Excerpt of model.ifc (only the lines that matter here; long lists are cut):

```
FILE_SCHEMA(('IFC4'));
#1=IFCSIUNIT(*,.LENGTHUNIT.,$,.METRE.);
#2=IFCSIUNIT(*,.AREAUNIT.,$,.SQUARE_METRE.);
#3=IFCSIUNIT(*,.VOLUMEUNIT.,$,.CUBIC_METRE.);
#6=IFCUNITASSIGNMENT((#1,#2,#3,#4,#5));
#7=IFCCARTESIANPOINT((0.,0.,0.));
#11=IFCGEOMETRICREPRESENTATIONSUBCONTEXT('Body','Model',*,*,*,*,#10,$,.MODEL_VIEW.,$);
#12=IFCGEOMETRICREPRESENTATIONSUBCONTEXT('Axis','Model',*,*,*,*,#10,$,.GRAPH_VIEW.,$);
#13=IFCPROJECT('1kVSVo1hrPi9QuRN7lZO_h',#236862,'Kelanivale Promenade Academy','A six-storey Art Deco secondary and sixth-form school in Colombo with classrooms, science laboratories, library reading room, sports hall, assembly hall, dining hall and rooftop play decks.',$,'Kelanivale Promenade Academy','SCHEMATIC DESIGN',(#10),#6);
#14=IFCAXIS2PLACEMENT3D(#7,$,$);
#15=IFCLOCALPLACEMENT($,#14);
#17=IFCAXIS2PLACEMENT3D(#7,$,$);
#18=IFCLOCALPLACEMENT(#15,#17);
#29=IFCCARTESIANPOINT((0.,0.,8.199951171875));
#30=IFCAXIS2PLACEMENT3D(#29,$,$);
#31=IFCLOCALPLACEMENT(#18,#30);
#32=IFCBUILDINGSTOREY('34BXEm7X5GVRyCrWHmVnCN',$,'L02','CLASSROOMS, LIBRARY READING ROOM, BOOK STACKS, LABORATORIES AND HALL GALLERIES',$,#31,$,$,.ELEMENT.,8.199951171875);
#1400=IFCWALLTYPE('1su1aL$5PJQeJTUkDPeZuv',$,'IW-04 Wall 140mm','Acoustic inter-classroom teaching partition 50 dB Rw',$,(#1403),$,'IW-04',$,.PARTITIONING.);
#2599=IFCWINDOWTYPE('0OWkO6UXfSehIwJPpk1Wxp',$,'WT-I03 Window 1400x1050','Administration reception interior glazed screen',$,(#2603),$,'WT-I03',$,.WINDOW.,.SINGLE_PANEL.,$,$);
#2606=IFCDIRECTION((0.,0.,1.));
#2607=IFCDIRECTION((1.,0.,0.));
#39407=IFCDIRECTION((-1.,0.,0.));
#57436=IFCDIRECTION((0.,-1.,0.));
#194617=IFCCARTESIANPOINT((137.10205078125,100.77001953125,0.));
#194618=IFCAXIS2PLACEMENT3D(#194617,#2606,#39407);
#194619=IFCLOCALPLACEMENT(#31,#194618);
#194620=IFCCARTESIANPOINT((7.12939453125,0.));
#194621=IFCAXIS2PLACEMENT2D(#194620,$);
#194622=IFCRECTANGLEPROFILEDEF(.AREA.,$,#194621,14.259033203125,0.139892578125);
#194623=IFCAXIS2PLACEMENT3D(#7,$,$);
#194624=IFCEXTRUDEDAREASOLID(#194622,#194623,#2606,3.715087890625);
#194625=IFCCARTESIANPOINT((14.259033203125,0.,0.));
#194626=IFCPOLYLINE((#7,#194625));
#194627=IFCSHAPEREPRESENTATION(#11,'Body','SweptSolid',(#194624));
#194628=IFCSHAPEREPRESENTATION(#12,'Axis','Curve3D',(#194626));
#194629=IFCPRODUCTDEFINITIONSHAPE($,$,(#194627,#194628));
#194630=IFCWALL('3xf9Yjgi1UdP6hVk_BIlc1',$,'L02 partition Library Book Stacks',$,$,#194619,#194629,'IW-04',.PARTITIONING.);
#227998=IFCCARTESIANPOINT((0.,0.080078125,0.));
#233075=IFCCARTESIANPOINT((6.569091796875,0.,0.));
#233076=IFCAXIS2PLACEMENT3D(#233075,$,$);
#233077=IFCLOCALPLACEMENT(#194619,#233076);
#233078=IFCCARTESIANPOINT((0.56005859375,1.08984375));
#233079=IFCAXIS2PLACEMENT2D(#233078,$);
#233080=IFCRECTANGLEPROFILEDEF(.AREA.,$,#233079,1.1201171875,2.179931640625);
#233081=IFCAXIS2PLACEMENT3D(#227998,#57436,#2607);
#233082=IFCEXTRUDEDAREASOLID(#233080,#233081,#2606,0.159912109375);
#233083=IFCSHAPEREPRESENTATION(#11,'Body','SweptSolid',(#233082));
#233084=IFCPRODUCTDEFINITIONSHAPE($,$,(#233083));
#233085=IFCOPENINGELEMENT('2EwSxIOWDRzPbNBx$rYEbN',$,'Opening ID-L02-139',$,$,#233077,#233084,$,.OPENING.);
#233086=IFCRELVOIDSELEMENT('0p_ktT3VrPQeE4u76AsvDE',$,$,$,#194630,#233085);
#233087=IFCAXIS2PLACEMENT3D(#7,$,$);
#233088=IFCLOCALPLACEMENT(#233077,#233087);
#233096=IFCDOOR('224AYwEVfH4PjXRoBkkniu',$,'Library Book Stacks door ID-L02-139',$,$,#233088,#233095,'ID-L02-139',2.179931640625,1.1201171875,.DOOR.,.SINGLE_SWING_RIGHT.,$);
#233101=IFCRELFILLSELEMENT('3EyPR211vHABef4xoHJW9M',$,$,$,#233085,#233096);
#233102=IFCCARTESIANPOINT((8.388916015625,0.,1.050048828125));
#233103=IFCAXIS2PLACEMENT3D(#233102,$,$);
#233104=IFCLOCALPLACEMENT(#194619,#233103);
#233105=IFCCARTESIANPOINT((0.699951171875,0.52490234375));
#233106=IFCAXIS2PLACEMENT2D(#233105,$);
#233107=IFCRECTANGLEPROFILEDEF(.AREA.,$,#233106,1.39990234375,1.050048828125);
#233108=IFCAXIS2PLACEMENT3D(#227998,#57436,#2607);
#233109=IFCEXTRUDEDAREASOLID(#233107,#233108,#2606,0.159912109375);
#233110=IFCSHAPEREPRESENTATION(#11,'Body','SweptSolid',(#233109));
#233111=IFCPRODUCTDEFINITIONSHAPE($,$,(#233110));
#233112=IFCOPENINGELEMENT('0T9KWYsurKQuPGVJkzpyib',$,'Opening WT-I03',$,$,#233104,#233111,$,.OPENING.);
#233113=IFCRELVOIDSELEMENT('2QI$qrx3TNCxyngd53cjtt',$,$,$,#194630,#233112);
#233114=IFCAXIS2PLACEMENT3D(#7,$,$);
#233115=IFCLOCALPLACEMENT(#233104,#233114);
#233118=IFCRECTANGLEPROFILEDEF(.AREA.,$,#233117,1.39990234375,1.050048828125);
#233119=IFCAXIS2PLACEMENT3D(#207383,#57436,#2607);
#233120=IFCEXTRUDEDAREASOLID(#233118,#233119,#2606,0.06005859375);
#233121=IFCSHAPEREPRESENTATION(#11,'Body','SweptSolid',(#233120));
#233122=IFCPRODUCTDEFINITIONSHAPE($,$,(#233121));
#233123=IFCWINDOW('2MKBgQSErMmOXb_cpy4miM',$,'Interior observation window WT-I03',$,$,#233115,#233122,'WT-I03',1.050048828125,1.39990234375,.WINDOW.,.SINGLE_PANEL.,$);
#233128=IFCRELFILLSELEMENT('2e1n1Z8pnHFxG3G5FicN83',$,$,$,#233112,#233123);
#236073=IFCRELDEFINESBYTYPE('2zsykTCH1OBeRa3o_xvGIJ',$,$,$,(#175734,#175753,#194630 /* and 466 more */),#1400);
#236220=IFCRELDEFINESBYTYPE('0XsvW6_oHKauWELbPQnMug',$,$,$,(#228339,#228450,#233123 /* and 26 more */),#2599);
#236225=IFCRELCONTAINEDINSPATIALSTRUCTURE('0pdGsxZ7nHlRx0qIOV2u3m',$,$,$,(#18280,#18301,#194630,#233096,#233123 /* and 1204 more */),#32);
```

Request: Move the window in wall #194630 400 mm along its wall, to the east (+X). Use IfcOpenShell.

```python
import ifcopenshell
import ifcopenshell.api.geometry
import ifcopenshell.util.placement
import ifcopenshell.util.unit

model = ifcopenshell.open("model.ifc")
unit_scale = ifcopenshell.util.unit.calculate_unit_scale(model)

window = model.by_guid("2MKBgQSErMmOXb_cpy4miM")
opening = window.FillsVoids[0].RelatingOpeningElement
wall = opening.VoidsElements[0].RelatingBuildingElement

wall_matrix = ifcopenshell.util.placement.get_local_placement(wall.ObjectPlacement)
shift = wall_matrix[:3, 0] * -0.4 / unit_scale
before = ifcopenshell.util.placement.get_local_placement(window.ObjectPlacement)[:3, 3].copy()

# The window is placed relative to its opening, so it follows when the opening moves.
matrix = ifcopenshell.util.placement.get_local_placement(opening.ObjectPlacement)
matrix[:3, 3] += shift
ifcopenshell.api.geometry.edit_object_placement(
    model, product=opening, matrix=matrix, is_si=False, should_transform_children=True
)

after = ifcopenshell.util.placement.get_local_placement(window.ObjectPlacement)[:3, 3]
print("window moved by", (after - before).round(3) + 0.0)

model.write("model_rev.ifc")
```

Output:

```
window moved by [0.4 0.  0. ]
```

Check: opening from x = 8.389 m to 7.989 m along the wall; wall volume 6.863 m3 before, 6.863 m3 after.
